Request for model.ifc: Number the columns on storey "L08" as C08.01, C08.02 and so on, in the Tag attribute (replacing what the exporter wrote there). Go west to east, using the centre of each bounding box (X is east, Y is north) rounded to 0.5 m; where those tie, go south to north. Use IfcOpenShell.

First a look at what the model holds.

```python
import ifcopenshell
import ifcopenshell.util.element
import ifcopenshell.util.placement

model = ifcopenshell.open("model.ifc")
print(model.schema)
storey = next(s for s in model.by_type("IfcBuildingStorey") if s.Name == "L08")
columns = [e for e in ifcopenshell.util.element.get_decomposition(storey) if e.is_a("IfcColumn")]
for e in sorted(columns, key=lambda e: e.id()):
    origin = ifcopenshell.util.placement.get_local_placement(e.ObjectPlacement)[:3, 3]
    print(e.id(), e.Tag, e.Name, origin.round(2) + 0.0, sep=" | ")
```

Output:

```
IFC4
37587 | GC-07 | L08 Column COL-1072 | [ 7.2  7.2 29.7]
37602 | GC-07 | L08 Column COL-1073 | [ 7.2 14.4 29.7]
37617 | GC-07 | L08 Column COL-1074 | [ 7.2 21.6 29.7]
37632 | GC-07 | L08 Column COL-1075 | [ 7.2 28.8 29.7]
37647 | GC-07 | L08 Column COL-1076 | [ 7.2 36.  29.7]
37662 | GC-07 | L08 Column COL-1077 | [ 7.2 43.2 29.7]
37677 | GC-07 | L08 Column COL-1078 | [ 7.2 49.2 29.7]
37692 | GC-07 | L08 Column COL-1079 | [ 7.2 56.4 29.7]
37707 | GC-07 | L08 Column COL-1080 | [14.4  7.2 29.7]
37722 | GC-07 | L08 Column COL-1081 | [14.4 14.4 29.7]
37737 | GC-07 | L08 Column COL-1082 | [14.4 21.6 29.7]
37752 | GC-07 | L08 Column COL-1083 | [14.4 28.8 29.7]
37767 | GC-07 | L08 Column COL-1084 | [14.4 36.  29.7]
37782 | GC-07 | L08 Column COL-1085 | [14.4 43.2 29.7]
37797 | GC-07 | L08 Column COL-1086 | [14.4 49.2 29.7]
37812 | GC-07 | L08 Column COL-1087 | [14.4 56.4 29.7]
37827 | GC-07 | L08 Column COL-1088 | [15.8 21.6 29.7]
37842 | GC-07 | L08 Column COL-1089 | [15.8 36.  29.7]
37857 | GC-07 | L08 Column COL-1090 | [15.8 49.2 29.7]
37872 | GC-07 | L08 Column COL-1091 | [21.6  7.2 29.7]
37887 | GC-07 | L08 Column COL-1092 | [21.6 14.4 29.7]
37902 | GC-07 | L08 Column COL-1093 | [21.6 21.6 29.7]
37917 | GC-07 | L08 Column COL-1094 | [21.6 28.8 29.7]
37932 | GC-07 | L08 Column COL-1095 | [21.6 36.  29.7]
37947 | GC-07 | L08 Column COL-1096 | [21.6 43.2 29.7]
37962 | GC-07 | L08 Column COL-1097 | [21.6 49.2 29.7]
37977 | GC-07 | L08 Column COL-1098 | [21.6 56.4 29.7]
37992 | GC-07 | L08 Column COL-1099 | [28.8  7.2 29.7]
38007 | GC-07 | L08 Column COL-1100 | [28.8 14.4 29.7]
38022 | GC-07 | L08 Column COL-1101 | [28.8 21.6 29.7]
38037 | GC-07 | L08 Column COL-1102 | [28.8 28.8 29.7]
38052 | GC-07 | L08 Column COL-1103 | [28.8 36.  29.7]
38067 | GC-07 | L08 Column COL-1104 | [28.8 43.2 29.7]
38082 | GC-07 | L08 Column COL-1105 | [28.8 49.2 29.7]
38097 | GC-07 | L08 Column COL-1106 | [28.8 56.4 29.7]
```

```python
import ifcopenshell
import ifcopenshell.geom
import ifcopenshell.util.element
import ifcopenshell.util.shape

model = ifcopenshell.open("model.ifc")
settings = ifcopenshell.geom.settings()
settings.set("use-world-coords", True)


def centre(element):
    shape = ifcopenshell.geom.create_shape(settings, element)
    return ifcopenshell.util.shape.get_bbox_centroid(shape.geometry)


storey = next(s for s in model.by_type("IfcBuildingStorey") if s.Name == "L08")
columns = [e for e in ifcopenshell.util.element.get_decomposition(storey) if e.is_a("IfcColumn")]

# Insertion points can sit at a corner or the storey origin, so sort by the geometry (in metres).
centres = {e: centre(e) for e in columns}
columns.sort(key=lambda e: (round(centres[e][0] / 0.5), centres[e][1]))

for i, e in enumerate(columns, start=1):
    number = f"C08.{i:02d}"
    e.Tag = number
    print(e.id(), number)

model.write("model_edited.ifc")
```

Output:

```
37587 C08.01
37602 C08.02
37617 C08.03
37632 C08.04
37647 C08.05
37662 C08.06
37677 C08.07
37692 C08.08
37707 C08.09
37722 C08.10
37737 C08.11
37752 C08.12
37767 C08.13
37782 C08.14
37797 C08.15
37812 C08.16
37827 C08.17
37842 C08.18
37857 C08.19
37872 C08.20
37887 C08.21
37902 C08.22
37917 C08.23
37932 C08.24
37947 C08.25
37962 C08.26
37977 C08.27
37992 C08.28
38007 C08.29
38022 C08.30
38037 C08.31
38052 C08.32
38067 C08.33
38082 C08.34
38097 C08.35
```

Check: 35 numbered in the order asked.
